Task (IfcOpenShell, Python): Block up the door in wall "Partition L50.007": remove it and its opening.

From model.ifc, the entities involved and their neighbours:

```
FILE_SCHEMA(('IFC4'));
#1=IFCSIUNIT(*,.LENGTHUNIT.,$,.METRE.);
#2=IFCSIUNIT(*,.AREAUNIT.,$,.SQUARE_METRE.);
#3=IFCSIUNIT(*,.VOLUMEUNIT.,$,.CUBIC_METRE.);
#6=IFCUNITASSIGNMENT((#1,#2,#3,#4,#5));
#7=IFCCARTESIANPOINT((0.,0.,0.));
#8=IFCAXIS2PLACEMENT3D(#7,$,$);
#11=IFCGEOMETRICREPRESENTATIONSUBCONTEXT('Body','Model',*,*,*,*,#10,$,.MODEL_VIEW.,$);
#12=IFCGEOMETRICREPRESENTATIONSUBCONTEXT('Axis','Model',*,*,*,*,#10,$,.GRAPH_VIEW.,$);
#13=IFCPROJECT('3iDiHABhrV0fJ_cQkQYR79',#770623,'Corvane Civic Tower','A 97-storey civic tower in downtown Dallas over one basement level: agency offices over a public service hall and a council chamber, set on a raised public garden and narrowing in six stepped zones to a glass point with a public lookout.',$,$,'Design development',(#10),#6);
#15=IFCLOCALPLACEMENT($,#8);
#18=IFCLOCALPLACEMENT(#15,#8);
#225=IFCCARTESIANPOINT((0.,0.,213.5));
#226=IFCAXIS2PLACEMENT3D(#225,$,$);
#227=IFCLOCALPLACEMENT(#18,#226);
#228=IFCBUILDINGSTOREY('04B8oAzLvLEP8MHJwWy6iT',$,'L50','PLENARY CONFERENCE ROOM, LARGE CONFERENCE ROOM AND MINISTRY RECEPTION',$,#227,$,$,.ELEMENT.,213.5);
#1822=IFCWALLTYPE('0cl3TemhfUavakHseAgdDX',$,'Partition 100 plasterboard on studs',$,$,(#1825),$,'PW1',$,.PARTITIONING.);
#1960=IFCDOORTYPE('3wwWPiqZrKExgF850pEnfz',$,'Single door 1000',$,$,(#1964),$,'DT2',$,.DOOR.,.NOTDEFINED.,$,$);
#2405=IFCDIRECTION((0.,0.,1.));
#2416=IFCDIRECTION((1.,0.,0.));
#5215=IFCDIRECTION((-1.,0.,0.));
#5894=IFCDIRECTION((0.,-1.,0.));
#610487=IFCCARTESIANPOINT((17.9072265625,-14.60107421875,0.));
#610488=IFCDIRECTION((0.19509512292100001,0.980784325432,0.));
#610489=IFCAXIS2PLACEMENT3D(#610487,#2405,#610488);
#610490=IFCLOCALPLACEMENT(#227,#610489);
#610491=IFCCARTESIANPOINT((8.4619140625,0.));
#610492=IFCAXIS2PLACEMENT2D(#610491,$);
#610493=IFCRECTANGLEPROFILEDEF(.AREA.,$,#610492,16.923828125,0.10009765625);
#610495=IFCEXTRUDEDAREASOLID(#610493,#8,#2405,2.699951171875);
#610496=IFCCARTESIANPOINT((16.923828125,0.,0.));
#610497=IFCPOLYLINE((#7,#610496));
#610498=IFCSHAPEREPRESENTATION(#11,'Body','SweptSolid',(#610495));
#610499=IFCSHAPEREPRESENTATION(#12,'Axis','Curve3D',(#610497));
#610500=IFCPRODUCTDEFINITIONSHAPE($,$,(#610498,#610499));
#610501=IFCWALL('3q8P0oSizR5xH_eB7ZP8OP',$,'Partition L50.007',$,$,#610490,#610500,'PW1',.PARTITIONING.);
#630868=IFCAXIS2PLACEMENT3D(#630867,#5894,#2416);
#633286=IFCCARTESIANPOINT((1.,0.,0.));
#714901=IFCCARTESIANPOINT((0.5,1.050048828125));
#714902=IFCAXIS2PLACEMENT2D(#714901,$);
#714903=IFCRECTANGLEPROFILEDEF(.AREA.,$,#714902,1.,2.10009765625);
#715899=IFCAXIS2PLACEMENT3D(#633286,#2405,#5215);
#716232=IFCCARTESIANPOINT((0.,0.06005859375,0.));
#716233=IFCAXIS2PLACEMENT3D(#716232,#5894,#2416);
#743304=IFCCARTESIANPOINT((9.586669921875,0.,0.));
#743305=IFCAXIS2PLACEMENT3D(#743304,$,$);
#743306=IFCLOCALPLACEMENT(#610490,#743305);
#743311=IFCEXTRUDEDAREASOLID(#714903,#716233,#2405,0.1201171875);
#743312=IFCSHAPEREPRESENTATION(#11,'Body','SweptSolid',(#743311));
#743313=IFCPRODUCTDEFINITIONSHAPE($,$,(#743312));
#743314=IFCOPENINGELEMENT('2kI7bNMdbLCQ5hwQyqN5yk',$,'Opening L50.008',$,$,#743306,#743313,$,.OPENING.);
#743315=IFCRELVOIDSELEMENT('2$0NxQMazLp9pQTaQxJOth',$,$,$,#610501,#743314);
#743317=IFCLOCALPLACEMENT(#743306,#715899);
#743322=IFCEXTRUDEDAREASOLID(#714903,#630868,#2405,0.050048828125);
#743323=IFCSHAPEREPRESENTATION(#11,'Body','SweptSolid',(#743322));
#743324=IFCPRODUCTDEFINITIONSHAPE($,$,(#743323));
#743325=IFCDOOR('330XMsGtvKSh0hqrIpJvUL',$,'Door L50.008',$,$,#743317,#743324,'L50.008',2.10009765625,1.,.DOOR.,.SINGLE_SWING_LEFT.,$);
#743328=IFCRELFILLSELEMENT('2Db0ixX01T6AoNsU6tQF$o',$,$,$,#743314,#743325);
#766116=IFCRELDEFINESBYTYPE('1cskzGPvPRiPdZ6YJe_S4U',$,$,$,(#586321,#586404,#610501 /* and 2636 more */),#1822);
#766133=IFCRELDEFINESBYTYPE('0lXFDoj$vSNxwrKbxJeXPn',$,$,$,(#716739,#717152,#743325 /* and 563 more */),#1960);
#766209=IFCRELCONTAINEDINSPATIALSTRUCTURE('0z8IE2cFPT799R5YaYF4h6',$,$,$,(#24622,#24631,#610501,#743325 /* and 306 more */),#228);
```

```python
import ifcopenshell
import ifcopenshell.api.feature
import ifcopenshell.api.root
import ifcopenshell.geom
import ifcopenshell.util.shape

model = ifcopenshell.open("model.ifc")
settings = ifcopenshell.geom.settings()


def volume(element):
    """Net volume in cubic metres, openings subtracted."""
    shape = ifcopenshell.geom.create_shape(settings, element)
    return ifcopenshell.util.shape.get_volume(shape.geometry)


door = model.by_id(743325)
opening = door.FillsVoids[0].RelatingOpeningElement
wall = opening.VoidsElements[0].RelatingBuildingElement
before = volume(wall)

ifcopenshell.api.root.remove_product(model, product=door)
ifcopenshell.api.feature.remove_feature(model, feature=opening)

after = volume(wall)

print(f"wall volume {before:.3f} -> {after:.3f} m3")

model.write("model_v2.ifc")
```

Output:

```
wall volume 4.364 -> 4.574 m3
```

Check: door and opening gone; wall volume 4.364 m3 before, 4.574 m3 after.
